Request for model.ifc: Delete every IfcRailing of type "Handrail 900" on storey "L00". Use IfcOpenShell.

First a look at what the model holds.

```python
import ifcopenshell
import ifcopenshell.util.element

model = ifcopenshell.open("model.ifc")
print(model.schema)
storey = next(s for s in model.by_type("IfcBuildingStorey") if s.Name == "L00")
railings = [e for e in ifcopenshell.util.element.get_decomposition(storey) if e.is_a("IfcRailing")]
seen = {}
for e in railings:
    element_type = ifcopenshell.util.element.get_type(e)
    name = element_type.Name if element_type not in (None, e) else None
    seen[name] = seen.get(name, 0) + 1
for name, count in sorted(seen.items(), key=str):
    print(count, "x", name)
```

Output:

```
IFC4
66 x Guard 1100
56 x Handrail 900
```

```python
import ifcopenshell
import ifcopenshell.api.root
import ifcopenshell.util.element

model = ifcopenshell.open("model.ifc")

storey = next(s for s in model.by_type("IfcBuildingStorey") if s.Name == "L00")
railings = [e for e in ifcopenshell.util.element.get_decomposition(storey) if e.is_a("IfcRailing")]
targets = [e for e in railings if (t := ifcopenshell.util.element.get_type(e)) not in (None, e) and t.Name == "Handrail 900"]

for e in targets:
    ifcopenshell.api.root.remove_product(model, product=e)
print(len(targets), "removed")

model.write("model-out.ifc")
```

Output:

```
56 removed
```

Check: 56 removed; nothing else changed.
